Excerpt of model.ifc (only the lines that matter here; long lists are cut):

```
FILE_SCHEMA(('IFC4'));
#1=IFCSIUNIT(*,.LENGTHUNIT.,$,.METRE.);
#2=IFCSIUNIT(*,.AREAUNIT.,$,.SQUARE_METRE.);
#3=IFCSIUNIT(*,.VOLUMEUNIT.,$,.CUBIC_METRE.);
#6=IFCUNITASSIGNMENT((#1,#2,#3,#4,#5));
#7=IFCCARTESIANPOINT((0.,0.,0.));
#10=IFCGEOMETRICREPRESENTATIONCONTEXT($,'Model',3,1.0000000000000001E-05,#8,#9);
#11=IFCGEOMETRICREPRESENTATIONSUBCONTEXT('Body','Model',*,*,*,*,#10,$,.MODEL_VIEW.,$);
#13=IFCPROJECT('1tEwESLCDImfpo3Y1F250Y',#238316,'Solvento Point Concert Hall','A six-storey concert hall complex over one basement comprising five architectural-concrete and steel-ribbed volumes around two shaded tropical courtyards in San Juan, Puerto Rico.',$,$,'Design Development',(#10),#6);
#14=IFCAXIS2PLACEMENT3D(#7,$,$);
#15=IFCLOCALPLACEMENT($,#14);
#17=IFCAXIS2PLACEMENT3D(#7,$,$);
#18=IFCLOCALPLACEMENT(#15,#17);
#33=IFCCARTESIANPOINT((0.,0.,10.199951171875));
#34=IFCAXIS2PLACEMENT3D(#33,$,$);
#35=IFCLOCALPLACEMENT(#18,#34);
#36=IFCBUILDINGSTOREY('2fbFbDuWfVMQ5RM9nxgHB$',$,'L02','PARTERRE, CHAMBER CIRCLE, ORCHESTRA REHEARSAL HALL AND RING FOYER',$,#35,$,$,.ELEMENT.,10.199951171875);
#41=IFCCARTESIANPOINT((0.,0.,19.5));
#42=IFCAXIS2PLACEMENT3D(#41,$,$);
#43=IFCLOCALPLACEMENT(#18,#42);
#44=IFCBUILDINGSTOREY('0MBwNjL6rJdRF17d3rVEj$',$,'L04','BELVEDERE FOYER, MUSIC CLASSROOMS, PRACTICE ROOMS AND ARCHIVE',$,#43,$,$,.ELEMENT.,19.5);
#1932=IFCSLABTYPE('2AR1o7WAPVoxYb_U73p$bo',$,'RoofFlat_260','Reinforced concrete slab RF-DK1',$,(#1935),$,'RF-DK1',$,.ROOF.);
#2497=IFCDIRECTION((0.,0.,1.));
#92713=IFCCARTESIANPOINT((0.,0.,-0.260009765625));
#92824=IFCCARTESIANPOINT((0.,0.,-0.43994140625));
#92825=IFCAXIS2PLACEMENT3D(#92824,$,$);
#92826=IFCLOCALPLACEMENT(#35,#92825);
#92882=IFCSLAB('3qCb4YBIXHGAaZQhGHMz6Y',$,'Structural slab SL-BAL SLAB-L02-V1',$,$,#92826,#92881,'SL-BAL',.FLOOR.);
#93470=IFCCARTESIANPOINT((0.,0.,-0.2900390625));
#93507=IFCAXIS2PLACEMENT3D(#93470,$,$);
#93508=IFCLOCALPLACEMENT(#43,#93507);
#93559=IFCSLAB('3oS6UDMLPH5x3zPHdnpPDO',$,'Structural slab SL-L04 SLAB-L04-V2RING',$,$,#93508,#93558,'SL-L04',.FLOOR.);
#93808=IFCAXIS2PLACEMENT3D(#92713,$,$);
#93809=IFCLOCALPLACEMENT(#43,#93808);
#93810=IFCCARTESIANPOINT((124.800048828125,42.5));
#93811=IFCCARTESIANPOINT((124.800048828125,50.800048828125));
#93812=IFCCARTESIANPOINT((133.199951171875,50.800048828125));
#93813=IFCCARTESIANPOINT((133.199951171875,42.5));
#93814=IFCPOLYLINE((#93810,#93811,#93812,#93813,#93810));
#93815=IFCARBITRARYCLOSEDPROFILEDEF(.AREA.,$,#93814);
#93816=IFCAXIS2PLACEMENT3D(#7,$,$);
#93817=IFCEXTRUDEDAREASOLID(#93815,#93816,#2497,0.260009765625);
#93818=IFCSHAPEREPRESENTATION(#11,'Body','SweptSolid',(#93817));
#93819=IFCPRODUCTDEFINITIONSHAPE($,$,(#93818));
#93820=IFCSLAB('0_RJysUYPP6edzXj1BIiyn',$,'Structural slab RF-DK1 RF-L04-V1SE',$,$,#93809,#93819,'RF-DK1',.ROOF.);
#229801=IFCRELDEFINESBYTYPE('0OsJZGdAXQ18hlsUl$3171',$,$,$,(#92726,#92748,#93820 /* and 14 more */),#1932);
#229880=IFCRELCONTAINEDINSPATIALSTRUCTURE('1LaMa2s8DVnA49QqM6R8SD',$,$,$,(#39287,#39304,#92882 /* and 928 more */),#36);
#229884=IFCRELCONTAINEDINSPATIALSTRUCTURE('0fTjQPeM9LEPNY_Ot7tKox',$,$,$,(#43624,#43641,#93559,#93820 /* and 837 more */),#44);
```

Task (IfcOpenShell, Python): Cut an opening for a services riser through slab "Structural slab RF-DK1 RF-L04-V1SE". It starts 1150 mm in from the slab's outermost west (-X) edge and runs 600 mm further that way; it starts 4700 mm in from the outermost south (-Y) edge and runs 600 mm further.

```python
import numpy as np
import ifcopenshell
import ifcopenshell.api.feature
import ifcopenshell.api.geometry
import ifcopenshell.api.root
import ifcopenshell.geom
import ifcopenshell.util.placement
import ifcopenshell.util.representation
import ifcopenshell.util.shape
import ifcopenshell.util.unit

model = ifcopenshell.open("model.ifc")
unit_scale = ifcopenshell.util.unit.calculate_unit_scale(model)
settings = ifcopenshell.geom.settings()


def volume(element):
    """Net volume in cubic metres, openings subtracted."""
    shape = ifcopenshell.geom.create_shape(settings, element)
    return ifcopenshell.util.shape.get_volume(shape.geometry)


slab = model.by_guid("0_RJysUYPP6edzXj1BIiyn")
before = volume(slab)

# Extent in the slab's own axes, in metres. The edges named are its -X and -Y sides.
slab_shape = ifcopenshell.geom.create_shape(settings, slab)
vertices = ifcopenshell.util.shape.get_vertices(slab_shape.geometry)
x_min, y_min, bottom = vertices.min(axis=0)
top = vertices[:, 2].max()

opening = ifcopenshell.api.root.create_entity(model, ifc_class="IfcOpeningElement", name="Services riser opening", predefined_type="OPENING")
context = ifcopenshell.util.representation.get_context(model, "Model", "Body", "MODEL_VIEW")
width, depth = 0.6, 0.6
outline = [(0.0, 0.0), (width, 0.0), (width, depth), (0.0, depth), (0.0, 0.0)]
# Overshoot both faces by 50 mm so the cut is clean.
shape = ifcopenshell.api.geometry.add_slab_representation(
    model, context=context, depth=top - bottom + 0.1, polyline=outline
)
ifcopenshell.api.geometry.assign_representation(model, product=opening, representation=shape)

matrix = ifcopenshell.util.placement.get_local_placement(slab.ObjectPlacement)
matrix[:, 3] = matrix @ np.append(np.array([x_min + 1.15, y_min + 4.7, bottom - 0.05]) / unit_scale, 1.0)
ifcopenshell.api.geometry.edit_object_placement(model, product=opening, matrix=matrix, is_si=False)
ifcopenshell.api.feature.add_feature(model, feature=opening, element=slab)

after = volume(slab)

print(f"slab volume {before:.3f} -> {after:.3f} m3")

model.write("model_rev.ifc")
```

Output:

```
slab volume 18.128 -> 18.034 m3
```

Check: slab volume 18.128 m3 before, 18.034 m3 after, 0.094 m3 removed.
